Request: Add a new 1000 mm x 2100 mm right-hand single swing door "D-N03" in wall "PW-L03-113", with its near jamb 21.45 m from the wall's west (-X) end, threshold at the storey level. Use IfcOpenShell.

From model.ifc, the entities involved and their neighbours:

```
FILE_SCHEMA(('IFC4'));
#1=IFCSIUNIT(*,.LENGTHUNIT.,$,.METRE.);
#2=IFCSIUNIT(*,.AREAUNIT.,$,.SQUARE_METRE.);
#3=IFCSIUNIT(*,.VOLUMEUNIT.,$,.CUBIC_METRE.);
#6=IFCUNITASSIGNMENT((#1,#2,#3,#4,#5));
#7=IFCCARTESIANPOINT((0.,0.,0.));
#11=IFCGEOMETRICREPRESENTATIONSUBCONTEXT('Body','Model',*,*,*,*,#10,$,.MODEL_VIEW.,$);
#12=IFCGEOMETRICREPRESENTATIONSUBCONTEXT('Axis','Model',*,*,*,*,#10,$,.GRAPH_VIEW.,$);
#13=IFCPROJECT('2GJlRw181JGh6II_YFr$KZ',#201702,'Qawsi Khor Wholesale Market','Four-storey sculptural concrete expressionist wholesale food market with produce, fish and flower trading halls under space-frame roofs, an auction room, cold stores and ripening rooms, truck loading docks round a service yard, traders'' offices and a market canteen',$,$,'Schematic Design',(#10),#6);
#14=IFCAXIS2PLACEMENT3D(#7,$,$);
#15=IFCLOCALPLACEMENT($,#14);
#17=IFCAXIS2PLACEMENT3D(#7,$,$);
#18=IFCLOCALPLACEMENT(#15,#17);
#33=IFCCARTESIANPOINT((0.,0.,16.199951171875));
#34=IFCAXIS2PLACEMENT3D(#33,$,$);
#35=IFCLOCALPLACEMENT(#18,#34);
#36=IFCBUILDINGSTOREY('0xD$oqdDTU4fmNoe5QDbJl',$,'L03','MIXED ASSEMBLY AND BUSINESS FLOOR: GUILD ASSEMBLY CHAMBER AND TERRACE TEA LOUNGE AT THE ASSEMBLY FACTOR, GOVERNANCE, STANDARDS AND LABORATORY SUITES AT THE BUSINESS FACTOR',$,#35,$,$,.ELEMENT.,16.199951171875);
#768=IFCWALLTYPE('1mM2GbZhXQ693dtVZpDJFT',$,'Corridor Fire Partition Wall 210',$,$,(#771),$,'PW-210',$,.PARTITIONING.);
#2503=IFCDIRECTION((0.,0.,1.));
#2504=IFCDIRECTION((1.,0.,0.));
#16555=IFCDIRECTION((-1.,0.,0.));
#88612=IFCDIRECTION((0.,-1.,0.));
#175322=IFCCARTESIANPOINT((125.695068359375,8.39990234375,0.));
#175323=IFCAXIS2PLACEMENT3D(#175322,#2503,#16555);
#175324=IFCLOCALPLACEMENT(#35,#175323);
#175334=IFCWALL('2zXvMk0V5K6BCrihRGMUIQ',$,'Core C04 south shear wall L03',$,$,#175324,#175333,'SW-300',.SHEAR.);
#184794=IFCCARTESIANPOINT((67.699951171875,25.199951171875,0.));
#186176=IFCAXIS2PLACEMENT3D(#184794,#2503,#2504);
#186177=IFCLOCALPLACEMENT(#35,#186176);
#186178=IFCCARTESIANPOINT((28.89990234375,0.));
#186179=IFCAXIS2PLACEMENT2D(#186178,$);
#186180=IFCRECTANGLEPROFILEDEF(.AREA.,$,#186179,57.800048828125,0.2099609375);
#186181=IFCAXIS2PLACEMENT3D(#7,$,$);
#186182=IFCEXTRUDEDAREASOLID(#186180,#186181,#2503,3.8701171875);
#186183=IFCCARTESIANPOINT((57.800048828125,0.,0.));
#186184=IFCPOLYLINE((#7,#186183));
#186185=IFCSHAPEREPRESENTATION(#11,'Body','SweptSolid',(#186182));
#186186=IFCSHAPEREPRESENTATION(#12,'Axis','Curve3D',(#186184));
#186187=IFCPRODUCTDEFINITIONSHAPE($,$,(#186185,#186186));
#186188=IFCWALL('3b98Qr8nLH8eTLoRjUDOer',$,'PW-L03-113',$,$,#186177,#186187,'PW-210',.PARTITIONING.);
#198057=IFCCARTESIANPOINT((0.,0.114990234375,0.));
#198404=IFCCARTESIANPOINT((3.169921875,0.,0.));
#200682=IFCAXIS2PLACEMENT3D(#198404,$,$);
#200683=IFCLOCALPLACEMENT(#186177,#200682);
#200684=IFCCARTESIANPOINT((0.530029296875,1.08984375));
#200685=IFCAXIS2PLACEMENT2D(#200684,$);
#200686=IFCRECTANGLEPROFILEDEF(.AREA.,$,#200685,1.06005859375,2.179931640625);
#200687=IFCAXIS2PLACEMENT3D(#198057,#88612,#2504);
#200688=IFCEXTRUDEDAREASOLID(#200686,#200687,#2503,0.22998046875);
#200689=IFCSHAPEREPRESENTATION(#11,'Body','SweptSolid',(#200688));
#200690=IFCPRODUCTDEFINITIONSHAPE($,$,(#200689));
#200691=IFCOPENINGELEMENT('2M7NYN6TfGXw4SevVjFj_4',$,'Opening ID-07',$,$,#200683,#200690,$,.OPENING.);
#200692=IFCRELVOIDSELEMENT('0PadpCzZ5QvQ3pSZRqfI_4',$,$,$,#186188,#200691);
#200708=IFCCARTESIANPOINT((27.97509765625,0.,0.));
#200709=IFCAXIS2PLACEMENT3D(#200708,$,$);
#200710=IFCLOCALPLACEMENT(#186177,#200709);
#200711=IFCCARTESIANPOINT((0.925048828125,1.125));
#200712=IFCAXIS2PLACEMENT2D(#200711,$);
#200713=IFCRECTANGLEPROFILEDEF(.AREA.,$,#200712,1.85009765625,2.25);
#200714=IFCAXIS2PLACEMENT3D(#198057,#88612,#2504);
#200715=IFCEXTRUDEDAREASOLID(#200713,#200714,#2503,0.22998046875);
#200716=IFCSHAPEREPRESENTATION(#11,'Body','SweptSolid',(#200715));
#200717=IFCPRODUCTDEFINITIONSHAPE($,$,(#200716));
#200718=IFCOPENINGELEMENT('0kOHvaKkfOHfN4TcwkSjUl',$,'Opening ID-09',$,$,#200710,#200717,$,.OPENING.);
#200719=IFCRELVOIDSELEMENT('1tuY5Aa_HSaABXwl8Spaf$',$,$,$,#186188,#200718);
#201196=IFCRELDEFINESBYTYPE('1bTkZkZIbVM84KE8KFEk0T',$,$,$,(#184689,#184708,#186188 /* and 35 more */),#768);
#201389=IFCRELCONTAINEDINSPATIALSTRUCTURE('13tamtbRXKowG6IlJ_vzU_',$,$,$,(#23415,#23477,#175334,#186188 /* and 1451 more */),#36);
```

```python
import numpy as np
import ifcopenshell
import ifcopenshell.api.feature
import ifcopenshell.api.geometry
import ifcopenshell.api.root
import ifcopenshell.api.spatial
import ifcopenshell.geom
import ifcopenshell.util.element
import ifcopenshell.util.placement
import ifcopenshell.util.representation
import ifcopenshell.util.shape
import ifcopenshell.util.unit

model = ifcopenshell.open("model.ifc")
unit_scale = ifcopenshell.util.unit.calculate_unit_scale(model)
settings = ifcopenshell.geom.settings()


def volume(element):
    """Net volume in cubic metres, openings subtracted."""
    shape = ifcopenshell.geom.create_shape(settings, element)
    return ifcopenshell.util.shape.get_volume(shape.geometry)


wall = model.by_guid("3b98Qr8nLH8eTLoRjUDOer")
storey = ifcopenshell.util.element.get_container(wall, ifc_class="IfcBuildingStorey")
context = ifcopenshell.util.representation.get_context(model, "Model", "Body", "MODEL_VIEW")
before = volume(wall)

width, height, from_end, sill = 1, 2.1, 21.45, 0.0  # metres

# The wall runs along its own X axis, and the end named is its -X end.
wall_shape = ifcopenshell.geom.create_shape(settings, wall)
x, y, z = ifcopenshell.util.shape.get_vertices(wall_shape.geometry).T
start = x.min() + from_end
face, thickness = float(y.min()), float(y.max() - y.min())
wall_matrix = ifcopenshell.util.placement.get_local_placement(wall.ObjectPlacement)
level = ifcopenshell.util.placement.get_local_placement(storey.ObjectPlacement)[2, 3]


def in_wall(x, y):
    """Placement at x, y metres in the wall's axes, at sill height."""
    matrix = wall_matrix.copy()
    matrix[:, 3] = wall_matrix @ np.array([x / unit_scale, y / unit_scale, 0.0, 1.0])
    matrix[2, 3] = level + sill / unit_scale
    return matrix


# Opening: a box that overshoots both wall faces by 50 mm.
opening = ifcopenshell.api.root.create_entity(model, ifc_class="IfcOpeningElement", predefined_type="OPENING")
box = ifcopenshell.api.geometry.add_wall_representation(
    model, context=context, length=width, height=height, thickness=thickness + 0.1
)
ifcopenshell.api.geometry.assign_representation(model, product=opening, representation=box)
ifcopenshell.api.geometry.edit_object_placement(model, product=opening, matrix=in_wall(start, face - 0.05), is_si=False)
ifcopenshell.api.feature.add_feature(model, feature=opening, element=wall)

door = ifcopenshell.api.root.create_entity(model, ifc_class="IfcDoor", name="D-N03", predefined_type="DOOR")
door.OverallWidth, door.OverallHeight = width / unit_scale, height / unit_scale
door.OperationType = "SINGLE_SWING_RIGHT"
body = ifcopenshell.api.geometry.add_door_representation(
    model,
    context=context,
    overall_width=door.OverallWidth,
    overall_height=door.OverallHeight,
    operation_type="SINGLE_SWING_RIGHT",
    lining_properties={"LiningDepth": thickness / unit_scale, "ThresholdDepth": thickness / unit_scale},
)
ifcopenshell.api.geometry.assign_representation(model, product=door, representation=body)
ifcopenshell.api.spatial.assign_container(model, products=[door], relating_structure=storey)
ifcopenshell.api.feature.add_filling(model, opening=opening, element=door)

# The lining spans the wall, so the door starts at the wall face.
ifcopenshell.api.geometry.edit_object_placement(model, product=door, matrix=in_wall(start, face), is_si=False)

after = volume(wall)

print(f"wall volume {before:.3f} -> {after:.3f} m3")

model.write("model_edited.ifc")
```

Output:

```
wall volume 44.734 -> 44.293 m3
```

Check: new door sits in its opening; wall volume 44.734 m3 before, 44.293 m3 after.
